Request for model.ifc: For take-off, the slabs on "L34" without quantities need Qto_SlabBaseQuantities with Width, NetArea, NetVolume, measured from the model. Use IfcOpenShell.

First a look at what the model holds.

```python
import ifcopenshell
import ifcopenshell.util.element
import ifcopenshell.util.unit

model = ifcopenshell.open("model.ifc")
print(model.schema)
for unit_type in ("LENGTHUNIT", "AREAUNIT", "VOLUMEUNIT"):
    print(unit_type, ifcopenshell.util.unit.calculate_unit_scale(model, unit_type))
storey = next(s for s in model.by_type("IfcBuildingStorey") if s.Name == "L34")
slabs = [e for e in ifcopenshell.util.element.get_decomposition(storey) if e.is_a("IfcSlab")]
for e in sorted(slabs, key=lambda e: e.id()):
    print(e.id(), e.is_a(), e.Name, list(ifcopenshell.util.element.get_psets(e, qtos_only=True)), sep=" | ")
```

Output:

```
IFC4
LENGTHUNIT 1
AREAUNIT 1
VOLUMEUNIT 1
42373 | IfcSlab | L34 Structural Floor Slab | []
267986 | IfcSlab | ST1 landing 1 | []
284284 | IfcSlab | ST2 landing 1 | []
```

```python
import ifcopenshell
import ifcopenshell.api.pset
import ifcopenshell.geom
import ifcopenshell.util.element
import ifcopenshell.util.shape
import ifcopenshell.util.unit

model = ifcopenshell.open("model.ifc")
unit_scale = ifcopenshell.util.unit.calculate_unit_scale(model)
area_scale = ifcopenshell.util.unit.calculate_unit_scale(model, "AREAUNIT")
volume_scale = ifcopenshell.util.unit.calculate_unit_scale(model, "VOLUMEUNIT")
settings = ifcopenshell.geom.settings()

storey = next(s for s in model.by_type("IfcBuildingStorey") if s.Name == "L34")
slabs = [e for e in ifcopenshell.util.element.get_decomposition(storey) if e.is_a("IfcSlab")]

for e in sorted(slabs, key=lambda e: e.id()):
    if ifcopenshell.util.element.get_psets(e, qtos_only=True, should_inherit=False):
        continue
    # Geometry comes back in metres, in the element's own axes.
    shape = ifcopenshell.geom.create_shape(settings, e)
    values = {
        "Width": ifcopenshell.util.shape.get_z(shape.geometry) / unit_scale,
        "NetArea": ifcopenshell.util.shape.get_footprint_area(shape.geometry) / area_scale,
        "NetVolume": ifcopenshell.util.shape.get_volume(shape.geometry) / volume_scale,
    }
    qto = ifcopenshell.api.pset.add_qto(model, product=e, name="Qto_SlabBaseQuantities")
    ifcopenshell.api.pset.edit_qto(model, qto=qto, properties=values)
    print(e.id(), {k: round(v, 3) for k, v in values.items()})

model.write("model_rev.ifc")
```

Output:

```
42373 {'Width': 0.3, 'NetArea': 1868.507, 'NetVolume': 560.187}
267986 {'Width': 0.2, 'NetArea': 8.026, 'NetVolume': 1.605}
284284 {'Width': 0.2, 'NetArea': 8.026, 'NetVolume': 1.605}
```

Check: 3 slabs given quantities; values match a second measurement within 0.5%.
